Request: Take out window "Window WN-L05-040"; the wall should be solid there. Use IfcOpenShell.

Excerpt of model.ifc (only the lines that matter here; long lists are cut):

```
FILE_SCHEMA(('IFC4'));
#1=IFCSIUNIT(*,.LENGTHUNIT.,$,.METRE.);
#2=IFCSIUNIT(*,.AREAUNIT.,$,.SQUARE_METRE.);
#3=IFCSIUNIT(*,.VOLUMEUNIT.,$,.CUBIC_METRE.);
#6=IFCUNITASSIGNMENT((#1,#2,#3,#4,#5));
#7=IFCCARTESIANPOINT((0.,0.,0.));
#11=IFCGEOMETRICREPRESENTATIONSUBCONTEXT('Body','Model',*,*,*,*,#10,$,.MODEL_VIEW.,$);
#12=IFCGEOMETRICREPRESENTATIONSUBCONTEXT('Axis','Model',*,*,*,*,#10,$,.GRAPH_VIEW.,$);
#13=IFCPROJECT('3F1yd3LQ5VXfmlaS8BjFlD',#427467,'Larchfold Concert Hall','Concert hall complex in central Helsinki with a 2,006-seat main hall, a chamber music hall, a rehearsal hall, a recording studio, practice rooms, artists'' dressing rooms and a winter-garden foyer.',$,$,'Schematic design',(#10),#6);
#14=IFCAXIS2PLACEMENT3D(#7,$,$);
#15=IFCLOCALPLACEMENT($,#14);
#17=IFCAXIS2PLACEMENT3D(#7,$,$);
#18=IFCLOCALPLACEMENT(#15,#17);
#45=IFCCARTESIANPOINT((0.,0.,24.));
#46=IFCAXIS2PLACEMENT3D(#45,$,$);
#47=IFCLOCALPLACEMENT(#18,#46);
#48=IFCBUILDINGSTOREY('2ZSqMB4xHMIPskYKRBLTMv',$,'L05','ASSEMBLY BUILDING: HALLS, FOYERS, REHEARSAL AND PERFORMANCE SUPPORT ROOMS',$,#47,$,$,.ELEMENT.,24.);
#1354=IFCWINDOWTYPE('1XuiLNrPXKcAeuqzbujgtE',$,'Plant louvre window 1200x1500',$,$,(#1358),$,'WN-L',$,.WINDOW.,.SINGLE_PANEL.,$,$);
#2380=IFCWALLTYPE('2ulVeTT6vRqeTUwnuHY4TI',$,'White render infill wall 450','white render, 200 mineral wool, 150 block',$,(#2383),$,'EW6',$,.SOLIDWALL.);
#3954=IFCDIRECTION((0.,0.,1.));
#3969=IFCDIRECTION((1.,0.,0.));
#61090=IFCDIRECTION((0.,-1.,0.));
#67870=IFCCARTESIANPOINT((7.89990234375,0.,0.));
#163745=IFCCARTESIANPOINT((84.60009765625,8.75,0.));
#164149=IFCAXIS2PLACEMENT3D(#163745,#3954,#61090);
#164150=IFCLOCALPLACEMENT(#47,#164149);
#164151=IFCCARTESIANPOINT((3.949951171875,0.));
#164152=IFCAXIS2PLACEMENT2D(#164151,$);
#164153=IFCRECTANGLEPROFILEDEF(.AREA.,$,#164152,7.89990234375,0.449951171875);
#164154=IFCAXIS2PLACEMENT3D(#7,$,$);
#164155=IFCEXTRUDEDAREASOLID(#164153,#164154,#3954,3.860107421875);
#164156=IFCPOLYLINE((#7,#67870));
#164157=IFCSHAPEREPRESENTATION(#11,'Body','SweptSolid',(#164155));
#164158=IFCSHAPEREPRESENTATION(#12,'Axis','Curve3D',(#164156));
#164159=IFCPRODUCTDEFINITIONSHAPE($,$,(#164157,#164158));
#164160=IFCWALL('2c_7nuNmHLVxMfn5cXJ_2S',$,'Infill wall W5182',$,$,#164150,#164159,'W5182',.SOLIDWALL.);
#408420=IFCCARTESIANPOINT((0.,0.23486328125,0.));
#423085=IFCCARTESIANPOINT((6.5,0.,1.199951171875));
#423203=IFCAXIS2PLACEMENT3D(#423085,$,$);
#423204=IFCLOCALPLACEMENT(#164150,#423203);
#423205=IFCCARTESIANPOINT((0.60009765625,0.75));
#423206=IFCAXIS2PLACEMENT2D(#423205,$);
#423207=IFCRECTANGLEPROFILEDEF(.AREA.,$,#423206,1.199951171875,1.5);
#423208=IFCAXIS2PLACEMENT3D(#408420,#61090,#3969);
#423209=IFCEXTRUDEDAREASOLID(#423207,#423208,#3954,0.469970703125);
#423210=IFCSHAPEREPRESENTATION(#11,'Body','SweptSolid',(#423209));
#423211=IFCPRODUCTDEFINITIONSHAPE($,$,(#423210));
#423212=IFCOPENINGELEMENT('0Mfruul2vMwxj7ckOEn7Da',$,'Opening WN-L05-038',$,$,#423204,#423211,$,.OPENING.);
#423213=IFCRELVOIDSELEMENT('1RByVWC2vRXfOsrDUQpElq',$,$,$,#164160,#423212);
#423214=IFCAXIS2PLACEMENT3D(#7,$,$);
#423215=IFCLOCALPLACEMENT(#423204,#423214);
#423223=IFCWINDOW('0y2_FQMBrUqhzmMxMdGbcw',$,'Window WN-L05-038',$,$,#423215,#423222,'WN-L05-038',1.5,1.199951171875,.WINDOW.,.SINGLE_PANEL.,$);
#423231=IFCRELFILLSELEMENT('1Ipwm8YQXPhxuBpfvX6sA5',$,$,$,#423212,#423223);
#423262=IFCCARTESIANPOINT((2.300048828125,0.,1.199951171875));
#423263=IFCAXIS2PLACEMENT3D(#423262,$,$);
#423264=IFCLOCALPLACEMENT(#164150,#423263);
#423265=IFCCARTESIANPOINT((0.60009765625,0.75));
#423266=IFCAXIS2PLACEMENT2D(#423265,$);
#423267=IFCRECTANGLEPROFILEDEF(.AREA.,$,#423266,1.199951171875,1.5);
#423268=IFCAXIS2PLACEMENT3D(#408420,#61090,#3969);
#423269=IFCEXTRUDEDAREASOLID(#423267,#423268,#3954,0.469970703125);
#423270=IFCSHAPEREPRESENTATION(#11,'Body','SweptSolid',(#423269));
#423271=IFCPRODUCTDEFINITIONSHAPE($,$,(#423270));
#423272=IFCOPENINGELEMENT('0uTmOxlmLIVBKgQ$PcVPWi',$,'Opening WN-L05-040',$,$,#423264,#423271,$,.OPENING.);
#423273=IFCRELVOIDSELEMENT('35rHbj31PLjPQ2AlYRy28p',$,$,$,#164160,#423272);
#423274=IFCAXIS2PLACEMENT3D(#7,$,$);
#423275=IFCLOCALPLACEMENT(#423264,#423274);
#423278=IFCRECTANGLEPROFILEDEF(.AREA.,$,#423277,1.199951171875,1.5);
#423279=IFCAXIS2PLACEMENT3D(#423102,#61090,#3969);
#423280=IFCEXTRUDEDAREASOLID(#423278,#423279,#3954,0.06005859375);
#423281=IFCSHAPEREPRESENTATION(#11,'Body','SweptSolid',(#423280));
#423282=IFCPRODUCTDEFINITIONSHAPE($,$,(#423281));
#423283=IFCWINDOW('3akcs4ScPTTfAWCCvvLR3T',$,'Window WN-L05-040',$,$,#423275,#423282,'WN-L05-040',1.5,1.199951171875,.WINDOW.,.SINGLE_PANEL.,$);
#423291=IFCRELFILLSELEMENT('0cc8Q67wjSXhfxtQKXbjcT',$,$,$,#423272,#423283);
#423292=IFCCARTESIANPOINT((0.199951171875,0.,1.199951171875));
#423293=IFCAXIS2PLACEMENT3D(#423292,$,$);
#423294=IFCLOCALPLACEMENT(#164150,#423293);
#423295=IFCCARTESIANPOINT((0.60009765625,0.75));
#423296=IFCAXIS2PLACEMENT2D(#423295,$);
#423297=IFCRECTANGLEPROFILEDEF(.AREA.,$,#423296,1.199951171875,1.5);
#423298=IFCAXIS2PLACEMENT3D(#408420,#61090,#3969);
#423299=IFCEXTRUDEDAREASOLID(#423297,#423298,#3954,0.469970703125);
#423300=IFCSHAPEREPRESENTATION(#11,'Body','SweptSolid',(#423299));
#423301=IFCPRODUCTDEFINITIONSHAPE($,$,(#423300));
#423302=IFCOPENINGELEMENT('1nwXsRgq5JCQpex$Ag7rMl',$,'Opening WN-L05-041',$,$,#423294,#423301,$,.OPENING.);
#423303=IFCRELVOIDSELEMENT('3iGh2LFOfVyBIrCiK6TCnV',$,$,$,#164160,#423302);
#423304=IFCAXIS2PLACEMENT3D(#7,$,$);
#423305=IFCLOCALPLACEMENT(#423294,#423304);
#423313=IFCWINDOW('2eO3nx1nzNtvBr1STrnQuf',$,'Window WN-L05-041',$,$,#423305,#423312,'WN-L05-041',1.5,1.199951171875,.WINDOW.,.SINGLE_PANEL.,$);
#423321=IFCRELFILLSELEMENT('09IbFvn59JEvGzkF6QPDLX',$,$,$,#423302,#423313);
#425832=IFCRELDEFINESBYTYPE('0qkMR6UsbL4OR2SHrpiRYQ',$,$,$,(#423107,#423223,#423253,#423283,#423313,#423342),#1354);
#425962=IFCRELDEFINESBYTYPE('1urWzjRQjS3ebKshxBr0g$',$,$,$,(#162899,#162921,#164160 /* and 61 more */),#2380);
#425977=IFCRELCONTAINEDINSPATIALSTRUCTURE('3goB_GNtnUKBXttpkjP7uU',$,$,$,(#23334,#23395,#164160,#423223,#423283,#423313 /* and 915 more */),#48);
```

```python
import ifcopenshell
import ifcopenshell.api.feature
import ifcopenshell.api.root
import ifcopenshell.geom
import ifcopenshell.util.shape

model = ifcopenshell.open("model.ifc")
settings = ifcopenshell.geom.settings()


def volume(element):
    """Net volume in cubic metres, openings subtracted."""
    shape = ifcopenshell.geom.create_shape(settings, element)
    return ifcopenshell.util.shape.get_volume(shape.geometry)


window = model.by_id(423283)
opening = window.FillsVoids[0].RelatingOpeningElement
wall = opening.VoidsElements[0].RelatingBuildingElement
before = volume(wall)

ifcopenshell.api.root.remove_product(model, product=window)
ifcopenshell.api.feature.remove_feature(model, feature=opening)

after = volume(wall)

print(f"wall volume {before:.3f} -> {after:.3f} m3")

model.write("model_updated.ifc")
```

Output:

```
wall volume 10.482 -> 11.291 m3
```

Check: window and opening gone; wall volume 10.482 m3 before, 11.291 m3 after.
